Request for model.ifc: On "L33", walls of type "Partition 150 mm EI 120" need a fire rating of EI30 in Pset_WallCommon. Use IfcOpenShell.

First a look at what the model holds.

```python
import ifcopenshell
import ifcopenshell.util.element

model = ifcopenshell.open("model.ifc")
print(model.schema)
storey = next(s for s in model.by_type("IfcBuildingStorey") if s.Name == "L33")
walls = [e for e in ifcopenshell.util.element.get_decomposition(storey) if e.is_a("IfcWall")]
seen = {}
for e in walls:
    element_type = ifcopenshell.util.element.get_type(e)
    key = (element_type.Name if element_type != e and element_type else None, ifcopenshell.util.element.get_pset(e, "Pset_WallCommon", "FireRating"))
    seen[key] = seen.get(key, 0) + 1
for (name, value), count in sorted(seen.items(), key=str):
    print(count, "x", name, "|", value)
```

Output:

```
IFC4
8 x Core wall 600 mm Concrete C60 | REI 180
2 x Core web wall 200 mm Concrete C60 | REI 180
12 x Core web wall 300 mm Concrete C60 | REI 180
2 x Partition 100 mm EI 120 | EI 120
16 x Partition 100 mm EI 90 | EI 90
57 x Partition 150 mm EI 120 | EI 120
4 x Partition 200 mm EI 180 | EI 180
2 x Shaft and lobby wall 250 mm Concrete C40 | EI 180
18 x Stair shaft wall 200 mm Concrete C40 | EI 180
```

```python
import ifcopenshell
import ifcopenshell.api.pset
import ifcopenshell.util.element

model = ifcopenshell.open("model.ifc")

storey = next(s for s in model.by_type("IfcBuildingStorey") if s.Name == "L33")
walls = [e for e in ifcopenshell.util.element.get_decomposition(storey) if e.is_a("IfcWall")]

count = 0
for e in walls:
    element_type = ifcopenshell.util.element.get_type(e)
    if element_type in (None, e) or element_type.Name != "Partition 150 mm EI 120":
        continue
    found = ifcopenshell.util.element.get_pset(e, "Pset_WallCommon", should_inherit=False)
    if found:
        pset = model.by_id(found["id"])
        if len(ifcopenshell.util.element.get_elements_by_pset(pset)) > 1:
            pset = ifcopenshell.api.pset.unshare_pset(model, products=[e], pset=pset)[0]
    else:
        pset = ifcopenshell.api.pset.add_pset(model, product=e, name="Pset_WallCommon")
    ifcopenshell.api.pset.edit_pset(model, pset=pset, properties={"FireRating": "EI30"})
    count += 1

print(count, "walls updated")

model.write("model-out.ifc")
```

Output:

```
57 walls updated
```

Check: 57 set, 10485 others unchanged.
